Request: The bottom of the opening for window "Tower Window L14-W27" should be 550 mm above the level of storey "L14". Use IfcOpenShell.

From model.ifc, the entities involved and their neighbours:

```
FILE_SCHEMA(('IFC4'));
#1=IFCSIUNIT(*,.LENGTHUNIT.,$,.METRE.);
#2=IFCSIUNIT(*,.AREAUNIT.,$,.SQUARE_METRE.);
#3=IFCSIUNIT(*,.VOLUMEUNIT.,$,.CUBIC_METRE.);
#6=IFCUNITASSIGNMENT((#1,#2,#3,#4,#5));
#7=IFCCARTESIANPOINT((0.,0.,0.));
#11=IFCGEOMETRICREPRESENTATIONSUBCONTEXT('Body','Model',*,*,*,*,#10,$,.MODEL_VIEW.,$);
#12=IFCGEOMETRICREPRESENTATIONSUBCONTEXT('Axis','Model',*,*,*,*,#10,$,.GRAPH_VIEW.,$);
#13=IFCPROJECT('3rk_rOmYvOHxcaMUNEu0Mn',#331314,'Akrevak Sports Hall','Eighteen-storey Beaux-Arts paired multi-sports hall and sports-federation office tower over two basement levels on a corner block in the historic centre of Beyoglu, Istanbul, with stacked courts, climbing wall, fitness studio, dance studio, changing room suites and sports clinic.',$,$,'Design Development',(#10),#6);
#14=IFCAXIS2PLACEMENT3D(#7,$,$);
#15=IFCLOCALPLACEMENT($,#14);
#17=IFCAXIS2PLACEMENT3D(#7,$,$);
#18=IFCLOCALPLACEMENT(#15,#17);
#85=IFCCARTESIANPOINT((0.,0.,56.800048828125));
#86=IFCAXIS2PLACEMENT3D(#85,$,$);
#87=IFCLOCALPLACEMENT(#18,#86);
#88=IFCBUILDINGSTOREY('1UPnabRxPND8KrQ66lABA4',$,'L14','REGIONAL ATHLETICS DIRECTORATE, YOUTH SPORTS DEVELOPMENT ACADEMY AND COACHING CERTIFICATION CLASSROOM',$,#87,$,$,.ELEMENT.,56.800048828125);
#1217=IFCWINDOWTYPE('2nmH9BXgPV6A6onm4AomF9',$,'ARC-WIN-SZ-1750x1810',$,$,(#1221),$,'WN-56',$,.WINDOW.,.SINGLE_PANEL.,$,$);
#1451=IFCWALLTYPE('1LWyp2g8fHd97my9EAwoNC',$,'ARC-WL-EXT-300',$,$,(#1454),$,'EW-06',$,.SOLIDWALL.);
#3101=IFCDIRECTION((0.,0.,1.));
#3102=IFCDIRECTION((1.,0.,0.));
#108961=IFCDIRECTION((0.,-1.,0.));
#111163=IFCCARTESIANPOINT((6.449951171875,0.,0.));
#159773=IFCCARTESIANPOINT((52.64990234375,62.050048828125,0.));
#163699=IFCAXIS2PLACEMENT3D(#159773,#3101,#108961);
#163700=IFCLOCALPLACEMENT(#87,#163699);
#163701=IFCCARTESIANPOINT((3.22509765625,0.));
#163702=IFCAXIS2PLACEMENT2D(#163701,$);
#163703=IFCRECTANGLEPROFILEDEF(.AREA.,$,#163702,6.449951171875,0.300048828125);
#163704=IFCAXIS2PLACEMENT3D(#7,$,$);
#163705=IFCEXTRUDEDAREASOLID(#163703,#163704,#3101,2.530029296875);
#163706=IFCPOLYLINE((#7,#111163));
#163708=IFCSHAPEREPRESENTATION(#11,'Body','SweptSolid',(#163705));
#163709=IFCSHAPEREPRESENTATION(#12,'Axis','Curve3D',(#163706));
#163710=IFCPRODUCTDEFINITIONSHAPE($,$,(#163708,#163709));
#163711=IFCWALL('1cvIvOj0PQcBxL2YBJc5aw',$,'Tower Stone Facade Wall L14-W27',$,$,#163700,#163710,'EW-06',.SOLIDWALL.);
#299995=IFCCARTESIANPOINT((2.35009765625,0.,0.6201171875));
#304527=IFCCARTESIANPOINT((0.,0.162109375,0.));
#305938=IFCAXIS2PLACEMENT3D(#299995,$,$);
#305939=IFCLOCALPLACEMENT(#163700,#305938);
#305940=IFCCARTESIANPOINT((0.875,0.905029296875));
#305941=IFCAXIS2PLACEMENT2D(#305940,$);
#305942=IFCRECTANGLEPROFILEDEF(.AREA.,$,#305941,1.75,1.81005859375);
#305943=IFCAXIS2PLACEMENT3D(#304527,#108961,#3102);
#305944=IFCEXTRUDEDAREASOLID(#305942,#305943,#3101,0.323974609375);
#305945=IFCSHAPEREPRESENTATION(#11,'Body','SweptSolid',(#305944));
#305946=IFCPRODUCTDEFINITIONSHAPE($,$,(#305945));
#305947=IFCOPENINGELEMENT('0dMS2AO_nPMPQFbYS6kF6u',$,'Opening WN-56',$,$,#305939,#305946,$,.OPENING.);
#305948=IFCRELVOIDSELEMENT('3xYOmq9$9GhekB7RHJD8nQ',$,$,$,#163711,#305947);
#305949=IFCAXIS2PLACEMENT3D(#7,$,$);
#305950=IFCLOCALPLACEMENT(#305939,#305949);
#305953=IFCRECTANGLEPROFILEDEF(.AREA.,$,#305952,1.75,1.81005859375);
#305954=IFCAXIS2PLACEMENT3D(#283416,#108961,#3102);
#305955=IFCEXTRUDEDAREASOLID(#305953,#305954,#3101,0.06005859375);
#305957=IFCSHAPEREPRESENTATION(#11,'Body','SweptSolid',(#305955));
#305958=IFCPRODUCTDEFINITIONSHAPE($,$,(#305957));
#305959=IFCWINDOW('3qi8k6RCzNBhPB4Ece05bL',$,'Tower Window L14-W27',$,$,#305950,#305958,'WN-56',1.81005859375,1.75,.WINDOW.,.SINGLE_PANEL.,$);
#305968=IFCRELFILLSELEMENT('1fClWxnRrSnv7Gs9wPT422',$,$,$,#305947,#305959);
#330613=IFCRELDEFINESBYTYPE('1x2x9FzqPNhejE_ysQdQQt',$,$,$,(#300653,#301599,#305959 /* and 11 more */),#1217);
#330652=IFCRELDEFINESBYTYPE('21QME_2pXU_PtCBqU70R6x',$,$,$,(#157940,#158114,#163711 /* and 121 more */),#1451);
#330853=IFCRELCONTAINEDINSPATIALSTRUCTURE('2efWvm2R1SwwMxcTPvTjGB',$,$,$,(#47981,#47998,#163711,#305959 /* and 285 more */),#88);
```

```python
import numpy as np
import ifcopenshell
import ifcopenshell.api.geometry
import ifcopenshell.geom
import ifcopenshell.util.element
import ifcopenshell.util.placement
import ifcopenshell.util.shape
import ifcopenshell.util.unit

model = ifcopenshell.open("model.ifc")
unit_scale = ifcopenshell.util.unit.calculate_unit_scale(model)

window = model.by_guid("3qi8k6RCzNBhPB4Ece05bL")
opening = window.FillsVoids[0].RelatingOpeningElement
storey = ifcopenshell.util.element.get_container(window, ifc_class="IfcBuildingStorey")
level = ifcopenshell.util.placement.get_local_placement(storey.ObjectPlacement)[2, 3]

# The opening's origin need not be at the sill, so measure its lowest point.
shape = ifcopenshell.geom.create_shape(ifcopenshell.geom.settings(), opening)
bottom = ifcopenshell.util.shape.get_shape_bottom_elevation(shape, shape.geometry) / unit_scale
dz = level + 0.55 / unit_scale - bottom

shift = np.array([0.0, 0.0, dz])
# The window is placed relative to its opening, so it follows when the opening moves.
matrix = ifcopenshell.util.placement.get_local_placement(opening.ObjectPlacement)
matrix[:3, 3] += shift
ifcopenshell.api.geometry.edit_object_placement(
    model, product=opening, matrix=matrix, is_si=False, should_transform_children=True
)

print(f"moved by {dz * unit_scale:+.3f} m")

model.write("model_rev.ifc")
```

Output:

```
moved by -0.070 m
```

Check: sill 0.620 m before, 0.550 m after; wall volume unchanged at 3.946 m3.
